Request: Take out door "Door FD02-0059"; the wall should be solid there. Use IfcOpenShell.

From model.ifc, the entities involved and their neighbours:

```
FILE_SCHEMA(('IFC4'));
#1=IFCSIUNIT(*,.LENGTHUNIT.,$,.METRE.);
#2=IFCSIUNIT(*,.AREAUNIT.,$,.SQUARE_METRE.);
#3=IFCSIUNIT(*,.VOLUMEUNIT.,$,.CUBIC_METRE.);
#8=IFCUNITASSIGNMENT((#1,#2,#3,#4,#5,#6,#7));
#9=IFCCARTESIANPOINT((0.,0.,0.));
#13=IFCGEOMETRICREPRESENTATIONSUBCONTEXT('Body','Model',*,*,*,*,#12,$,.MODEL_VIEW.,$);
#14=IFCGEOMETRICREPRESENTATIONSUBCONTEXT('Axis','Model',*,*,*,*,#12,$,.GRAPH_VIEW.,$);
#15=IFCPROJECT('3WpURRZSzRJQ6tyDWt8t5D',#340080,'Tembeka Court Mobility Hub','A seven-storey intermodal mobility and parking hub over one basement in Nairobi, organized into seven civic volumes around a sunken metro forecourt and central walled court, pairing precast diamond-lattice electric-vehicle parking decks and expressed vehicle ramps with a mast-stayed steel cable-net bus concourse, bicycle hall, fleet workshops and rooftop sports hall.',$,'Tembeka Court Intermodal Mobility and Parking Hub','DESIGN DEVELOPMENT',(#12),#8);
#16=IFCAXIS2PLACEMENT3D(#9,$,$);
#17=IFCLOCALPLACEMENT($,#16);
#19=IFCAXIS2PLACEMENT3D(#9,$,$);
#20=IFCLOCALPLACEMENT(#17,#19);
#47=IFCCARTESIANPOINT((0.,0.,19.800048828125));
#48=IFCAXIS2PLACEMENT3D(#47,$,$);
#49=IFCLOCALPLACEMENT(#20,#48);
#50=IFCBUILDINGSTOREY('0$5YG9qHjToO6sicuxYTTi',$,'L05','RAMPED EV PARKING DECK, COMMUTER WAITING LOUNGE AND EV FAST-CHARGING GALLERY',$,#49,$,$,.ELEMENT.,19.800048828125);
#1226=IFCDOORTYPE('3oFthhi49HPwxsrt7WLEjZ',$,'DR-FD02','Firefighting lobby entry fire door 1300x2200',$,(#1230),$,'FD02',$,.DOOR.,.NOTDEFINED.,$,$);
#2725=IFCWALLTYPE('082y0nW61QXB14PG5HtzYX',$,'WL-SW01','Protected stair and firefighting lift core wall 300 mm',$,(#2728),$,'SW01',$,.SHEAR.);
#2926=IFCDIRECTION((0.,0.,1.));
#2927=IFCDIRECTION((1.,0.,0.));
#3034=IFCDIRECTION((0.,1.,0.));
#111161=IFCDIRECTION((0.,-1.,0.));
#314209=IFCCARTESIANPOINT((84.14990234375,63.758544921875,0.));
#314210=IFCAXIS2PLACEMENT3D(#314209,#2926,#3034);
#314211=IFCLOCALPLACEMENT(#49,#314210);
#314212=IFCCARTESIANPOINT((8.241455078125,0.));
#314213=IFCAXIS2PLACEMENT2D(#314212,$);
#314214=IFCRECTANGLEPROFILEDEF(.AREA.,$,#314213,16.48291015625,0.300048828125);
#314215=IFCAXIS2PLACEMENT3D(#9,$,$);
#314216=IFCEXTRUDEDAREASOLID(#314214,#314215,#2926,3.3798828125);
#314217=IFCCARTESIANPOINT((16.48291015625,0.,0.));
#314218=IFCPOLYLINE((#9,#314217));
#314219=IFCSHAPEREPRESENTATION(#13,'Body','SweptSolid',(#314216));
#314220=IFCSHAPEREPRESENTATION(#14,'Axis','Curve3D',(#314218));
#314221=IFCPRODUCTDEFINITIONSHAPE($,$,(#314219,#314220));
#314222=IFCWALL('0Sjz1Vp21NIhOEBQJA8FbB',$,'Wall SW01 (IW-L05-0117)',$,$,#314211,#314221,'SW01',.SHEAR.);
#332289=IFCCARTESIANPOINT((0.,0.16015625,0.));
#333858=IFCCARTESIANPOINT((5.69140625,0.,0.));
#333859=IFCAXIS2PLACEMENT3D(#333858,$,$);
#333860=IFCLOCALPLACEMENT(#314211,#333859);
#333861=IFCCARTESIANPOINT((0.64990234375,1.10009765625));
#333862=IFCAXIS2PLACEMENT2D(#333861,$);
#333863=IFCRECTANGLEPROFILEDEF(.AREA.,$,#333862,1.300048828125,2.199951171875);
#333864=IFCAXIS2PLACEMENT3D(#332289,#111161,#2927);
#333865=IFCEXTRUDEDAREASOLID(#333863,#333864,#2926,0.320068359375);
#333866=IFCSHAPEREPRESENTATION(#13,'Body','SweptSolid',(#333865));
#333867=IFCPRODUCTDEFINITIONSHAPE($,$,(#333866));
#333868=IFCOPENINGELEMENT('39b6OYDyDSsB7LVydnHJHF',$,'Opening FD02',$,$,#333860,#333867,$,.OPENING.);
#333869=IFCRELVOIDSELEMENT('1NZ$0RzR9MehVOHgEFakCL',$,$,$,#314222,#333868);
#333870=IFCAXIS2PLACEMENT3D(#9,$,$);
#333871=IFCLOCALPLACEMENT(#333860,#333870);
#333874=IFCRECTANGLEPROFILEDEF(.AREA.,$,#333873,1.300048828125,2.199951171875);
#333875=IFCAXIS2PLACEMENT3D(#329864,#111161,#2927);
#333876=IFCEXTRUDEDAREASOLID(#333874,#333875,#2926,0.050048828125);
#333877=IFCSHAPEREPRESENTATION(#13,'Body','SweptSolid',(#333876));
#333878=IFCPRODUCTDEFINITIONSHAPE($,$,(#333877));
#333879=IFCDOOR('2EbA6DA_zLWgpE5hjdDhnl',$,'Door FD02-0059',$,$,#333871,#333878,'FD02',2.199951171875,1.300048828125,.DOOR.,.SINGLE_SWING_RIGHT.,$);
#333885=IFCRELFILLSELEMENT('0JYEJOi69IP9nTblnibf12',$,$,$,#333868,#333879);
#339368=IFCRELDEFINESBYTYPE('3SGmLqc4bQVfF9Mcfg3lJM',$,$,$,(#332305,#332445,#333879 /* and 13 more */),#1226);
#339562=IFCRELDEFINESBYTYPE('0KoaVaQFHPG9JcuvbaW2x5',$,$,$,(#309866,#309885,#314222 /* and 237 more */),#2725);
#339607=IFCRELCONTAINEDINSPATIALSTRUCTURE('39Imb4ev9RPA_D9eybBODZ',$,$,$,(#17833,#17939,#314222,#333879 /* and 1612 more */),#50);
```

```python
import ifcopenshell
import ifcopenshell.api.feature
import ifcopenshell.api.root
import ifcopenshell.geom
import ifcopenshell.util.shape

model = ifcopenshell.open("model.ifc")
settings = ifcopenshell.geom.settings()


def volume(element):
    """Net volume in cubic metres, openings subtracted."""
    shape = ifcopenshell.geom.create_shape(settings, element)
    return ifcopenshell.util.shape.get_volume(shape.geometry)


door = model.by_guid("2EbA6DA_zLWgpE5hjdDhnl")
opening = door.FillsVoids[0].RelatingOpeningElement
wall = opening.VoidsElements[0].RelatingBuildingElement
before = volume(wall)

ifcopenshell.api.root.remove_product(model, product=door)
ifcopenshell.api.feature.remove_feature(model, feature=opening)

after = volume(wall)

print(f"wall volume {before:.3f} -> {after:.3f} m3")

model.write("model_updated.ifc")
```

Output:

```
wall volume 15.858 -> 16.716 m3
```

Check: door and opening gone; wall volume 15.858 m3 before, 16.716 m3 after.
